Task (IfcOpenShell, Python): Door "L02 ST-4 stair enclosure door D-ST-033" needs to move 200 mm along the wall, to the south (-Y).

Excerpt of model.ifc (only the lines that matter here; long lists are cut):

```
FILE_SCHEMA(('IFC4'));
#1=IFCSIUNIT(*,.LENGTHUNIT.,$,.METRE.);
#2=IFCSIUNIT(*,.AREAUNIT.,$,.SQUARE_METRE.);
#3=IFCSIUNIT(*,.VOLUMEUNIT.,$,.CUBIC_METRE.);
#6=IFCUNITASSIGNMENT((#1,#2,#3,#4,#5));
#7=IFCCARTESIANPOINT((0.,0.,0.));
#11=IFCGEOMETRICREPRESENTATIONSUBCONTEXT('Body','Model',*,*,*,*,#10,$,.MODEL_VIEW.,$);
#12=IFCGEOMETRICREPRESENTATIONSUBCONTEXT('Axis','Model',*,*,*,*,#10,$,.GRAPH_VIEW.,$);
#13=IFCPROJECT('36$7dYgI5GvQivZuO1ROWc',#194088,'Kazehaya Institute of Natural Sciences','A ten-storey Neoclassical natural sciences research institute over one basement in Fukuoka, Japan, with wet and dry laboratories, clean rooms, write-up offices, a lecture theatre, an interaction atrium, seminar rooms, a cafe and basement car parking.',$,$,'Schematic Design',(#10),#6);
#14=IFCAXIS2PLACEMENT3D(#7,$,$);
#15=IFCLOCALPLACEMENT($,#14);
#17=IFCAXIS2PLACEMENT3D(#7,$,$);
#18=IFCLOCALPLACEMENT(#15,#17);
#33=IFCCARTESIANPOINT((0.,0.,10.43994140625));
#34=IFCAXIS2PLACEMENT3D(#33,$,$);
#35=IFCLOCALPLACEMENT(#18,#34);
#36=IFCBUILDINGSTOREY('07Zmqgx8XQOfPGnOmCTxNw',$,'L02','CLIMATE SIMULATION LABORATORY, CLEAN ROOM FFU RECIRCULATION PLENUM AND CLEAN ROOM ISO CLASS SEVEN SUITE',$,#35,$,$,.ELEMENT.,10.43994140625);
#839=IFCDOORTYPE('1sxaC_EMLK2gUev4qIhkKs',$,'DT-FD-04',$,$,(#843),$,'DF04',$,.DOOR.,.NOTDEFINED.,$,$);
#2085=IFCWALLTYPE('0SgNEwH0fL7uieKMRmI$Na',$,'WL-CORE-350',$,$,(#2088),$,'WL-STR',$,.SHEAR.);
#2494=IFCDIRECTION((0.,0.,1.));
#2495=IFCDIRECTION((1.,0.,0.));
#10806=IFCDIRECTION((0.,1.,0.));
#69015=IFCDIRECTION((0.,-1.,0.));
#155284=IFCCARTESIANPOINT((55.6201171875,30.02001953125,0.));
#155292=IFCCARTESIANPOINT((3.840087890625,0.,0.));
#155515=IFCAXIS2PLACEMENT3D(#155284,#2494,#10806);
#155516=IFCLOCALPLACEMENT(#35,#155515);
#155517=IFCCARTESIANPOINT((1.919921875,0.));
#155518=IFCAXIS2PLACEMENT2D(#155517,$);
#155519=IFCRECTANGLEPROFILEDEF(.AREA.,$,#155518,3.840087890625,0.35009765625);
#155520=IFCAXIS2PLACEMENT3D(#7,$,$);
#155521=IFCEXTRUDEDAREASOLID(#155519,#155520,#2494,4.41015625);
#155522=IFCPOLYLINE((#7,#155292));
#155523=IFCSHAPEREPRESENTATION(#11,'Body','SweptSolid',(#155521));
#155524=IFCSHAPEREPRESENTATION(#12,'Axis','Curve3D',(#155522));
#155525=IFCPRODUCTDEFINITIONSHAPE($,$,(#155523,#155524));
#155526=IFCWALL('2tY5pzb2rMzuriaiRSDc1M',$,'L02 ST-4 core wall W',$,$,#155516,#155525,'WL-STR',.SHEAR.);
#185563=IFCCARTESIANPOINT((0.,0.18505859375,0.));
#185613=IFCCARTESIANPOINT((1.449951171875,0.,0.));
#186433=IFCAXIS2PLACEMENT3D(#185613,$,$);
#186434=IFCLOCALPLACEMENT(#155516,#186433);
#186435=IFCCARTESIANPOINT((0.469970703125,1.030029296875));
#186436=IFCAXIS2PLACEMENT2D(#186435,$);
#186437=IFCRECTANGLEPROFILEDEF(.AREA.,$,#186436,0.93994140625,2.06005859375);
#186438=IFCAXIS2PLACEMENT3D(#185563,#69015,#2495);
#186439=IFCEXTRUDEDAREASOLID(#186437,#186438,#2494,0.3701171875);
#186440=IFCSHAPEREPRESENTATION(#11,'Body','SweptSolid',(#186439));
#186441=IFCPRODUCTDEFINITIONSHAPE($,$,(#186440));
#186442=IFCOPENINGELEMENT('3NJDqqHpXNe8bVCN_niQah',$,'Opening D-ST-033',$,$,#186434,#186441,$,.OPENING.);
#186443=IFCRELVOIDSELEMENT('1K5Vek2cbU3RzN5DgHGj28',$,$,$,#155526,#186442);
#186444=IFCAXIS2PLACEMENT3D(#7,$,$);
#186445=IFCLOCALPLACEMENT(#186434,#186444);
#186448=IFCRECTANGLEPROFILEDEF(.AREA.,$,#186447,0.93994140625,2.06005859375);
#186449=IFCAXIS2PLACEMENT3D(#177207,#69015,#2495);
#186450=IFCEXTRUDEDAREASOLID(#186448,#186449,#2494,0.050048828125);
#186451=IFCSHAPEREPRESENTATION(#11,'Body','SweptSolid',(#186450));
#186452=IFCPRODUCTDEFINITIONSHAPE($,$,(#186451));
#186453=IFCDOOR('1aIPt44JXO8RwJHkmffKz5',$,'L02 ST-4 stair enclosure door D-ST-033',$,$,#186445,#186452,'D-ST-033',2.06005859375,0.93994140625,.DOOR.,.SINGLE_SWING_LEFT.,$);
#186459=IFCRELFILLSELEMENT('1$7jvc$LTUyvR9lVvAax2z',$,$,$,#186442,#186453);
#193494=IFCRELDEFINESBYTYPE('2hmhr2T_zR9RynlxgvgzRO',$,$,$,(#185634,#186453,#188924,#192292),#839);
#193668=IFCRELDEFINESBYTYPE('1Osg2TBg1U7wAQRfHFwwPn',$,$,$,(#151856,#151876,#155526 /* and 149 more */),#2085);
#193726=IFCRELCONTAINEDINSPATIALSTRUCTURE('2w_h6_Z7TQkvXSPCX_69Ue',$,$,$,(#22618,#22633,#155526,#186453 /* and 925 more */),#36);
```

```python
import ifcopenshell
import ifcopenshell.api.geometry
import ifcopenshell.util.placement
import ifcopenshell.util.unit

model = ifcopenshell.open("model.ifc")
unit_scale = ifcopenshell.util.unit.calculate_unit_scale(model)

door = model.by_id(186453)
opening = door.FillsVoids[0].RelatingOpeningElement
wall = opening.VoidsElements[0].RelatingBuildingElement

wall_matrix = ifcopenshell.util.placement.get_local_placement(wall.ObjectPlacement)
shift = wall_matrix[:3, 0] * -0.2 / unit_scale
before = ifcopenshell.util.placement.get_local_placement(door.ObjectPlacement)[:3, 3].copy()

# The door is placed relative to its opening, so it follows when the opening moves.
matrix = ifcopenshell.util.placement.get_local_placement(opening.ObjectPlacement)
matrix[:3, 3] += shift
ifcopenshell.api.geometry.edit_object_placement(
    model, product=opening, matrix=matrix, is_si=False, should_transform_children=True
)

after = ifcopenshell.util.placement.get_local_placement(door.ObjectPlacement)[:3, 3]
print("door moved by", (after - before).round(3) + 0.0)

model.write("model-out.ifc")
```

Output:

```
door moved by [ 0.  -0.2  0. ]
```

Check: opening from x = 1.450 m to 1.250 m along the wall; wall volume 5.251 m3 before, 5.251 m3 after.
